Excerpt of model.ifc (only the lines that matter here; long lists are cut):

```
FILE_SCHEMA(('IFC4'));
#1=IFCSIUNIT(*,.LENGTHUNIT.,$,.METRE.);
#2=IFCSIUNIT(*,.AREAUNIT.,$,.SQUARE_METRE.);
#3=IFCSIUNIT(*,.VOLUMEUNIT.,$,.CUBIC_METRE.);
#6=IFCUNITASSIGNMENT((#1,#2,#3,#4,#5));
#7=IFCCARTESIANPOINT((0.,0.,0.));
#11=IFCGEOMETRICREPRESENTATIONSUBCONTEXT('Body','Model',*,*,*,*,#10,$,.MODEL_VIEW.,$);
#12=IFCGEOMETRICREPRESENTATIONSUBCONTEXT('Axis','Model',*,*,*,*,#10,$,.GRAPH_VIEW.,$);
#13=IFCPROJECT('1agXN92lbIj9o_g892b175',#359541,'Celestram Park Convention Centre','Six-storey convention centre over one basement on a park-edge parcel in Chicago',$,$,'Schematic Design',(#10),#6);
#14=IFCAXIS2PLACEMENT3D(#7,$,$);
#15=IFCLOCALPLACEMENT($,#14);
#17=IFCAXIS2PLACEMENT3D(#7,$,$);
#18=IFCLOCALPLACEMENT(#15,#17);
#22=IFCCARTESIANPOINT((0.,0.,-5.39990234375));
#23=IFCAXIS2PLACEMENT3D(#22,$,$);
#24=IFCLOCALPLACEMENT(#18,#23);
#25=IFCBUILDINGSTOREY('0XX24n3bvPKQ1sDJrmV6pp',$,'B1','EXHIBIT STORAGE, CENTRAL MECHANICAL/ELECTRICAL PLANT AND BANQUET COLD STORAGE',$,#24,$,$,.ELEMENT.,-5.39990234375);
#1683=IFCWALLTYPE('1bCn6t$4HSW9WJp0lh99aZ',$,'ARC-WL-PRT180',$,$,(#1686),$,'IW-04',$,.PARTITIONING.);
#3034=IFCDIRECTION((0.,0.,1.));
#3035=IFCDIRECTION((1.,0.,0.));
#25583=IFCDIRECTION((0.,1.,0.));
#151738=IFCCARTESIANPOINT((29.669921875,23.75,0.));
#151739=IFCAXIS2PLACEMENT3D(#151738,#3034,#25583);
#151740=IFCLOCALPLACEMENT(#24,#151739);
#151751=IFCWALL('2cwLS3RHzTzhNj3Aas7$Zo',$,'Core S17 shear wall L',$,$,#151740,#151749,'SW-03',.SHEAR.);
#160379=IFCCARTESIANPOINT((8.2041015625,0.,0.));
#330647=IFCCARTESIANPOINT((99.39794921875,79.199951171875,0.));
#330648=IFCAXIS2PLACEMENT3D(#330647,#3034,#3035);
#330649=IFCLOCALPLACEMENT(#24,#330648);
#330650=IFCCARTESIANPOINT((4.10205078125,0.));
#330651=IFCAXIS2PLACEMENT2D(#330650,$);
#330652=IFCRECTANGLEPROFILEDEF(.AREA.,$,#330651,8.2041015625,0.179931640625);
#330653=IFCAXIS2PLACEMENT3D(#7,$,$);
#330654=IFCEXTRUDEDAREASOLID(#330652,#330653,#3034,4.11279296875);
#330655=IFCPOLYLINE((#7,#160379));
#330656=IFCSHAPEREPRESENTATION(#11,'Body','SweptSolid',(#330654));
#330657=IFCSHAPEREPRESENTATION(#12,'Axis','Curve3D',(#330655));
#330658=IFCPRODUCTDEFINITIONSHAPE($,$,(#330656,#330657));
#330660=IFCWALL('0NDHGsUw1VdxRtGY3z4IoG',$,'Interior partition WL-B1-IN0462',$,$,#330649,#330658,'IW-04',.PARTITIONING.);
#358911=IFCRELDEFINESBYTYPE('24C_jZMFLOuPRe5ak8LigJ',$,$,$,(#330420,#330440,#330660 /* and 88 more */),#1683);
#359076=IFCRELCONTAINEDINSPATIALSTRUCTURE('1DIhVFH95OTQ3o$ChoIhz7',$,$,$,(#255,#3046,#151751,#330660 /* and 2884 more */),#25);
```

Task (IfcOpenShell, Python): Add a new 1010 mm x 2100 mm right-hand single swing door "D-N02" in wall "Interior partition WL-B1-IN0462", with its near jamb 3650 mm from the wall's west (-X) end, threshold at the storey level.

```python
import numpy as np
import ifcopenshell
import ifcopenshell.api.feature
import ifcopenshell.api.geometry
import ifcopenshell.api.root
import ifcopenshell.api.spatial
import ifcopenshell.geom
import ifcopenshell.util.element
import ifcopenshell.util.placement
import ifcopenshell.util.representation
import ifcopenshell.util.shape
import ifcopenshell.util.unit

model = ifcopenshell.open("model.ifc")
unit_scale = ifcopenshell.util.unit.calculate_unit_scale(model)
settings = ifcopenshell.geom.settings()


def volume(element):
    """Net volume in cubic metres, openings subtracted."""
    shape = ifcopenshell.geom.create_shape(settings, element)
    return ifcopenshell.util.shape.get_volume(shape.geometry)


wall = model.by_guid("0NDHGsUw1VdxRtGY3z4IoG")
storey = ifcopenshell.util.element.get_container(wall, ifc_class="IfcBuildingStorey")
context = ifcopenshell.util.representation.get_context(model, "Model", "Body", "MODEL_VIEW")
before = volume(wall)

width, height, from_end, sill = 1.01, 2.1, 3.65, 0.0  # metres

# The wall runs along its own X axis, and the end named is its -X end.
wall_shape = ifcopenshell.geom.create_shape(settings, wall)
x, y, z = ifcopenshell.util.shape.get_vertices(wall_shape.geometry).T
start = x.min() + from_end
face, thickness = float(y.min()), float(y.max() - y.min())
wall_matrix = ifcopenshell.util.placement.get_local_placement(wall.ObjectPlacement)
level = ifcopenshell.util.placement.get_local_placement(storey.ObjectPlacement)[2, 3]


def in_wall(x, y):
    """Placement at x, y metres in the wall's axes, at sill height."""
    matrix = wall_matrix.copy()
    matrix[:, 3] = wall_matrix @ np.array([x / unit_scale, y / unit_scale, 0.0, 1.0])
    matrix[2, 3] = level + sill / unit_scale
    return matrix


# Opening: a box that overshoots both wall faces by 50 mm.
opening = ifcopenshell.api.root.create_entity(model, ifc_class="IfcOpeningElement", predefined_type="OPENING")
box = ifcopenshell.api.geometry.add_wall_representation(
    model, context=context, length=width, height=height, thickness=thickness + 0.1
)
ifcopenshell.api.geometry.assign_representation(model, product=opening, representation=box)
ifcopenshell.api.geometry.edit_object_placement(model, product=opening, matrix=in_wall(start, face - 0.05), is_si=False)
ifcopenshell.api.feature.add_feature(model, feature=opening, element=wall)

door = ifcopenshell.api.root.create_entity(model, ifc_class="IfcDoor", name="D-N02", predefined_type="DOOR")
door.OverallWidth, door.OverallHeight = width / unit_scale, height / unit_scale
door.OperationType = "SINGLE_SWING_RIGHT"
body = ifcopenshell.api.geometry.add_door_representation(
    model,
    context=context,
    overall_width=door.OverallWidth,
    overall_height=door.OverallHeight,
    operation_type="SINGLE_SWING_RIGHT",
    lining_properties={"LiningDepth": thickness / unit_scale, "ThresholdDepth": thickness / unit_scale},
)
ifcopenshell.api.geometry.assign_representation(model, product=door, representation=body)
ifcopenshell.api.spatial.assign_container(model, products=[door], relating_structure=storey)
ifcopenshell.api.feature.add_filling(model, opening=opening, element=door)

# The lining spans the wall, so the door starts at the wall face.
ifcopenshell.api.geometry.edit_object_placement(model, product=door, matrix=in_wall(start, face), is_si=False)

after = volume(wall)

print(f"wall volume {before:.3f} -> {after:.3f} m3")

model.write("model_v2.ifc")
```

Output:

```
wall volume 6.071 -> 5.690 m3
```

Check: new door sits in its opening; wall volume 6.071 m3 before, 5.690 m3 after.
